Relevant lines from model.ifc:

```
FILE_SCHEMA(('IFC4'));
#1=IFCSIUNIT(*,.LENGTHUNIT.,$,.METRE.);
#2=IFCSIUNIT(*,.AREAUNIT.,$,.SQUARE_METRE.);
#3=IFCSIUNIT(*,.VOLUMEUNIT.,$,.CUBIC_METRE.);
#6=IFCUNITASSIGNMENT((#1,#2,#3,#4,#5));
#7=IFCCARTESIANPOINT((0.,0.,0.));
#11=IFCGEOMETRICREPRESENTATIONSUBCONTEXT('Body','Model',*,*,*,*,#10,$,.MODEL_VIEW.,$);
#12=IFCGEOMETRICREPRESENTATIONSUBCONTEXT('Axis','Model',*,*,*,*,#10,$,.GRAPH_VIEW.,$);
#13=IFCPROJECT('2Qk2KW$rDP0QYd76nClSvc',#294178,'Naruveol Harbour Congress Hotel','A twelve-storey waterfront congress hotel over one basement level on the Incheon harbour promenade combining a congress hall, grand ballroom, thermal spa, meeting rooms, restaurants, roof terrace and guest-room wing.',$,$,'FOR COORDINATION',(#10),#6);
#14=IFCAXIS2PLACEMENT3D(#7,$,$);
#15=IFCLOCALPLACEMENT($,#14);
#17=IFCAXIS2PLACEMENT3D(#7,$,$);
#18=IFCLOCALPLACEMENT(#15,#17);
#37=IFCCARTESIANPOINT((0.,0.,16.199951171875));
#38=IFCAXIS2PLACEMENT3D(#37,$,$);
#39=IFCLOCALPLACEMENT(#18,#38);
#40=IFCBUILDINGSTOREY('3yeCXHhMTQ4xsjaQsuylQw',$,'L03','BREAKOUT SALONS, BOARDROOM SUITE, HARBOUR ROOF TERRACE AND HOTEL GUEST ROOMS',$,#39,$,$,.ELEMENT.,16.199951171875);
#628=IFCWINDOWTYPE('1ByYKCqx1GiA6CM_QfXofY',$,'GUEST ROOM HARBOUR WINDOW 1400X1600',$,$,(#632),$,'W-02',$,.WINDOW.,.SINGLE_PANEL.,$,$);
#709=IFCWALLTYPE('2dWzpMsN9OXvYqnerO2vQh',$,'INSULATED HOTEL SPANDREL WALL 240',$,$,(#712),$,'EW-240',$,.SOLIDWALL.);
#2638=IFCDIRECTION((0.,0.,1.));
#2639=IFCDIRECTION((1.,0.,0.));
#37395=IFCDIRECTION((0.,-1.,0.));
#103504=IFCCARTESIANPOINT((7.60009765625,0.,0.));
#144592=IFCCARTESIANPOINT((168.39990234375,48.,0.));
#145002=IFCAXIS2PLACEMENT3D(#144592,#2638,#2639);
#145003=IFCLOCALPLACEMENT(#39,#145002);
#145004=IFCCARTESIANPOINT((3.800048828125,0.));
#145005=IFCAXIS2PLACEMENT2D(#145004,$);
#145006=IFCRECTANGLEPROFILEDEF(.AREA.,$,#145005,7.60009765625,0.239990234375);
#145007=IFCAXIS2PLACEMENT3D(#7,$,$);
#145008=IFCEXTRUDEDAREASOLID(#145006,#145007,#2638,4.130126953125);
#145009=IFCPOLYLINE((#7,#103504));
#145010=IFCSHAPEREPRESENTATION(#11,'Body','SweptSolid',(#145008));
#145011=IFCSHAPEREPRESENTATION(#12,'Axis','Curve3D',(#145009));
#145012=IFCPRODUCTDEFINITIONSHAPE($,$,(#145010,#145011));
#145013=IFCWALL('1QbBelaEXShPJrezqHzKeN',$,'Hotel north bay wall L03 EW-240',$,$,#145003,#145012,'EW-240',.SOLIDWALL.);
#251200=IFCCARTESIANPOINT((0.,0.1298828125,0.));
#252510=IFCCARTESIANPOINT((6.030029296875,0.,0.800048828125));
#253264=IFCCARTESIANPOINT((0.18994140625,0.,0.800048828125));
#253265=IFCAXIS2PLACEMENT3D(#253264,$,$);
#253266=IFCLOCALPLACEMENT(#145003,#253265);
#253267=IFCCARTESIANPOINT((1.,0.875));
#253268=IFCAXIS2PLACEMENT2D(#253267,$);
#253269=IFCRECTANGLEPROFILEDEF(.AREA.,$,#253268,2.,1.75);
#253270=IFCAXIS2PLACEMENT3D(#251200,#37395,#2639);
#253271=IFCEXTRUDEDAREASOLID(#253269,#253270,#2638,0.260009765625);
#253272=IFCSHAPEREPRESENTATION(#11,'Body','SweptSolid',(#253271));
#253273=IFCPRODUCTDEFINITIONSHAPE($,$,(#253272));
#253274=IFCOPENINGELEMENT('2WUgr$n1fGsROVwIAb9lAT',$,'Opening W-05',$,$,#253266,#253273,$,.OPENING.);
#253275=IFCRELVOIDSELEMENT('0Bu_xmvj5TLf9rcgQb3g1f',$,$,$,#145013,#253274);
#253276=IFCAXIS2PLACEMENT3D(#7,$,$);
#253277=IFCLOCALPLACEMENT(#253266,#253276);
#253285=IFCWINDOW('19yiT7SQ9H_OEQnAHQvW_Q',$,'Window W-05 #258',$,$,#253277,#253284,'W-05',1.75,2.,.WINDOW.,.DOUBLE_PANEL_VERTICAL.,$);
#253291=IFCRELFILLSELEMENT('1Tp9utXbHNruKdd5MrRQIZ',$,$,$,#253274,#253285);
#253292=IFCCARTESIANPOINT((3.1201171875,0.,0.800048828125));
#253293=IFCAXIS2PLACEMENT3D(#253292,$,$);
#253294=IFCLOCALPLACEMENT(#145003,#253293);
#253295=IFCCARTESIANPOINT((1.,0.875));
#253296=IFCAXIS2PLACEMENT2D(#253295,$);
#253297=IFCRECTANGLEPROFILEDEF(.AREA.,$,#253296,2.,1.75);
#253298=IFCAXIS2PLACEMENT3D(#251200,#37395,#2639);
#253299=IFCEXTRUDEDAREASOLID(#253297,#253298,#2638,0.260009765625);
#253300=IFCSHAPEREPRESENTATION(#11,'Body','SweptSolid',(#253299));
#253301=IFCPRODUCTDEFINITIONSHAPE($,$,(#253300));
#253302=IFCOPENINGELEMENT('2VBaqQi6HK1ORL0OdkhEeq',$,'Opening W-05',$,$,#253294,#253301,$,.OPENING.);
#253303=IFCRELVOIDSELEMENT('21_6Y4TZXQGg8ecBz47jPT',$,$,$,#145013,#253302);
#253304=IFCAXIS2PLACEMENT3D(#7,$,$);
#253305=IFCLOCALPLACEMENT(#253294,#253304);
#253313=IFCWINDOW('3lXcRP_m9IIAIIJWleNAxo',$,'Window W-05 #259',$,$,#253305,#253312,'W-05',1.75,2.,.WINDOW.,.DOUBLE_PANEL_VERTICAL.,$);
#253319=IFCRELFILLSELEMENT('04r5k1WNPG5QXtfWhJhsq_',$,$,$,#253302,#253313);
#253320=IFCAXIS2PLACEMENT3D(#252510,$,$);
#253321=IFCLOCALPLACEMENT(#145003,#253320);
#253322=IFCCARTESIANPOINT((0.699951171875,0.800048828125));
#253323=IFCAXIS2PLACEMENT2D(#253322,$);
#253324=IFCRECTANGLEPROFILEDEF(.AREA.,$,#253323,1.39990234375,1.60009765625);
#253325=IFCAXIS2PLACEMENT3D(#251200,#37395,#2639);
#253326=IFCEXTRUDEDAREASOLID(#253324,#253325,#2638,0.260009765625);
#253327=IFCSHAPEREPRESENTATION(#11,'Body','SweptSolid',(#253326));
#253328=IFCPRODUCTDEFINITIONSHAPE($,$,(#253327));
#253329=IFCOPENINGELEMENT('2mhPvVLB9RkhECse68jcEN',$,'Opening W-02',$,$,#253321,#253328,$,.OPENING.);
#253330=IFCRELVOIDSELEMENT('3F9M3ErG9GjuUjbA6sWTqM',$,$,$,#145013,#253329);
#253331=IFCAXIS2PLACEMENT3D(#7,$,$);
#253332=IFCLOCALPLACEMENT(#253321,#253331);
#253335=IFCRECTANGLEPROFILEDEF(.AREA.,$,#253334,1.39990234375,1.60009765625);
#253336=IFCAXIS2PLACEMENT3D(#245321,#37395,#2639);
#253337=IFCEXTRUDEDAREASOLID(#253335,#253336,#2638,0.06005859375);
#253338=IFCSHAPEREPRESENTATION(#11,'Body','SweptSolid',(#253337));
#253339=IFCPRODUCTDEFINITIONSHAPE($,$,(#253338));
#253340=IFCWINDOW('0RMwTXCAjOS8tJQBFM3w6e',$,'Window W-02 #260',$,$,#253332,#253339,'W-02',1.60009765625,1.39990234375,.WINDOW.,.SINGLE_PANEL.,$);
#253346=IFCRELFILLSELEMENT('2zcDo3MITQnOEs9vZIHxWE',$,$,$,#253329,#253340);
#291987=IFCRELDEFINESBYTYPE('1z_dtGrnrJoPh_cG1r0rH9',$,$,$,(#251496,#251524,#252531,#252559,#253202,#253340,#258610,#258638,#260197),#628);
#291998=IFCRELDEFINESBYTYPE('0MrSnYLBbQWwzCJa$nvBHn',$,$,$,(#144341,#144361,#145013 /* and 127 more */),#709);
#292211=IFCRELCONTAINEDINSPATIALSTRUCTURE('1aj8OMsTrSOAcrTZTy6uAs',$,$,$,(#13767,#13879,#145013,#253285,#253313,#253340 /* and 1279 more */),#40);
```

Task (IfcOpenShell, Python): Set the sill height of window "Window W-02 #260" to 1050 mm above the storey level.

```python
import numpy as np
import ifcopenshell
import ifcopenshell.api.geometry
import ifcopenshell.geom
import ifcopenshell.util.element
import ifcopenshell.util.placement
import ifcopenshell.util.shape
import ifcopenshell.util.unit

model = ifcopenshell.open("model.ifc")
unit_scale = ifcopenshell.util.unit.calculate_unit_scale(model)

window = model.by_guid("0RMwTXCAjOS8tJQBFM3w6e")
opening = window.FillsVoids[0].RelatingOpeningElement
storey = ifcopenshell.util.element.get_container(window, ifc_class="IfcBuildingStorey")
level = ifcopenshell.util.placement.get_local_placement(storey.ObjectPlacement)[2, 3]

# The opening's origin need not be at the sill, so measure its lowest point.
shape = ifcopenshell.geom.create_shape(ifcopenshell.geom.settings(), opening)
bottom = ifcopenshell.util.shape.get_shape_bottom_elevation(shape, shape.geometry) / unit_scale
dz = level + 1.05 / unit_scale - bottom

shift = np.array([0.0, 0.0, dz])
# The window is placed relative to its opening, so it follows when the opening moves.
matrix = ifcopenshell.util.placement.get_local_placement(opening.ObjectPlacement)
matrix[:3, 3] += shift
ifcopenshell.api.geometry.edit_object_placement(
    model, product=opening, matrix=matrix, is_si=False, should_transform_children=True
)

print(f"moved by {dz * unit_scale:+.3f} m")

model.write("model_rev.ifc")
```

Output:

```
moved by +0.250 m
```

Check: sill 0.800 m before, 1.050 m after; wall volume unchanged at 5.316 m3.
